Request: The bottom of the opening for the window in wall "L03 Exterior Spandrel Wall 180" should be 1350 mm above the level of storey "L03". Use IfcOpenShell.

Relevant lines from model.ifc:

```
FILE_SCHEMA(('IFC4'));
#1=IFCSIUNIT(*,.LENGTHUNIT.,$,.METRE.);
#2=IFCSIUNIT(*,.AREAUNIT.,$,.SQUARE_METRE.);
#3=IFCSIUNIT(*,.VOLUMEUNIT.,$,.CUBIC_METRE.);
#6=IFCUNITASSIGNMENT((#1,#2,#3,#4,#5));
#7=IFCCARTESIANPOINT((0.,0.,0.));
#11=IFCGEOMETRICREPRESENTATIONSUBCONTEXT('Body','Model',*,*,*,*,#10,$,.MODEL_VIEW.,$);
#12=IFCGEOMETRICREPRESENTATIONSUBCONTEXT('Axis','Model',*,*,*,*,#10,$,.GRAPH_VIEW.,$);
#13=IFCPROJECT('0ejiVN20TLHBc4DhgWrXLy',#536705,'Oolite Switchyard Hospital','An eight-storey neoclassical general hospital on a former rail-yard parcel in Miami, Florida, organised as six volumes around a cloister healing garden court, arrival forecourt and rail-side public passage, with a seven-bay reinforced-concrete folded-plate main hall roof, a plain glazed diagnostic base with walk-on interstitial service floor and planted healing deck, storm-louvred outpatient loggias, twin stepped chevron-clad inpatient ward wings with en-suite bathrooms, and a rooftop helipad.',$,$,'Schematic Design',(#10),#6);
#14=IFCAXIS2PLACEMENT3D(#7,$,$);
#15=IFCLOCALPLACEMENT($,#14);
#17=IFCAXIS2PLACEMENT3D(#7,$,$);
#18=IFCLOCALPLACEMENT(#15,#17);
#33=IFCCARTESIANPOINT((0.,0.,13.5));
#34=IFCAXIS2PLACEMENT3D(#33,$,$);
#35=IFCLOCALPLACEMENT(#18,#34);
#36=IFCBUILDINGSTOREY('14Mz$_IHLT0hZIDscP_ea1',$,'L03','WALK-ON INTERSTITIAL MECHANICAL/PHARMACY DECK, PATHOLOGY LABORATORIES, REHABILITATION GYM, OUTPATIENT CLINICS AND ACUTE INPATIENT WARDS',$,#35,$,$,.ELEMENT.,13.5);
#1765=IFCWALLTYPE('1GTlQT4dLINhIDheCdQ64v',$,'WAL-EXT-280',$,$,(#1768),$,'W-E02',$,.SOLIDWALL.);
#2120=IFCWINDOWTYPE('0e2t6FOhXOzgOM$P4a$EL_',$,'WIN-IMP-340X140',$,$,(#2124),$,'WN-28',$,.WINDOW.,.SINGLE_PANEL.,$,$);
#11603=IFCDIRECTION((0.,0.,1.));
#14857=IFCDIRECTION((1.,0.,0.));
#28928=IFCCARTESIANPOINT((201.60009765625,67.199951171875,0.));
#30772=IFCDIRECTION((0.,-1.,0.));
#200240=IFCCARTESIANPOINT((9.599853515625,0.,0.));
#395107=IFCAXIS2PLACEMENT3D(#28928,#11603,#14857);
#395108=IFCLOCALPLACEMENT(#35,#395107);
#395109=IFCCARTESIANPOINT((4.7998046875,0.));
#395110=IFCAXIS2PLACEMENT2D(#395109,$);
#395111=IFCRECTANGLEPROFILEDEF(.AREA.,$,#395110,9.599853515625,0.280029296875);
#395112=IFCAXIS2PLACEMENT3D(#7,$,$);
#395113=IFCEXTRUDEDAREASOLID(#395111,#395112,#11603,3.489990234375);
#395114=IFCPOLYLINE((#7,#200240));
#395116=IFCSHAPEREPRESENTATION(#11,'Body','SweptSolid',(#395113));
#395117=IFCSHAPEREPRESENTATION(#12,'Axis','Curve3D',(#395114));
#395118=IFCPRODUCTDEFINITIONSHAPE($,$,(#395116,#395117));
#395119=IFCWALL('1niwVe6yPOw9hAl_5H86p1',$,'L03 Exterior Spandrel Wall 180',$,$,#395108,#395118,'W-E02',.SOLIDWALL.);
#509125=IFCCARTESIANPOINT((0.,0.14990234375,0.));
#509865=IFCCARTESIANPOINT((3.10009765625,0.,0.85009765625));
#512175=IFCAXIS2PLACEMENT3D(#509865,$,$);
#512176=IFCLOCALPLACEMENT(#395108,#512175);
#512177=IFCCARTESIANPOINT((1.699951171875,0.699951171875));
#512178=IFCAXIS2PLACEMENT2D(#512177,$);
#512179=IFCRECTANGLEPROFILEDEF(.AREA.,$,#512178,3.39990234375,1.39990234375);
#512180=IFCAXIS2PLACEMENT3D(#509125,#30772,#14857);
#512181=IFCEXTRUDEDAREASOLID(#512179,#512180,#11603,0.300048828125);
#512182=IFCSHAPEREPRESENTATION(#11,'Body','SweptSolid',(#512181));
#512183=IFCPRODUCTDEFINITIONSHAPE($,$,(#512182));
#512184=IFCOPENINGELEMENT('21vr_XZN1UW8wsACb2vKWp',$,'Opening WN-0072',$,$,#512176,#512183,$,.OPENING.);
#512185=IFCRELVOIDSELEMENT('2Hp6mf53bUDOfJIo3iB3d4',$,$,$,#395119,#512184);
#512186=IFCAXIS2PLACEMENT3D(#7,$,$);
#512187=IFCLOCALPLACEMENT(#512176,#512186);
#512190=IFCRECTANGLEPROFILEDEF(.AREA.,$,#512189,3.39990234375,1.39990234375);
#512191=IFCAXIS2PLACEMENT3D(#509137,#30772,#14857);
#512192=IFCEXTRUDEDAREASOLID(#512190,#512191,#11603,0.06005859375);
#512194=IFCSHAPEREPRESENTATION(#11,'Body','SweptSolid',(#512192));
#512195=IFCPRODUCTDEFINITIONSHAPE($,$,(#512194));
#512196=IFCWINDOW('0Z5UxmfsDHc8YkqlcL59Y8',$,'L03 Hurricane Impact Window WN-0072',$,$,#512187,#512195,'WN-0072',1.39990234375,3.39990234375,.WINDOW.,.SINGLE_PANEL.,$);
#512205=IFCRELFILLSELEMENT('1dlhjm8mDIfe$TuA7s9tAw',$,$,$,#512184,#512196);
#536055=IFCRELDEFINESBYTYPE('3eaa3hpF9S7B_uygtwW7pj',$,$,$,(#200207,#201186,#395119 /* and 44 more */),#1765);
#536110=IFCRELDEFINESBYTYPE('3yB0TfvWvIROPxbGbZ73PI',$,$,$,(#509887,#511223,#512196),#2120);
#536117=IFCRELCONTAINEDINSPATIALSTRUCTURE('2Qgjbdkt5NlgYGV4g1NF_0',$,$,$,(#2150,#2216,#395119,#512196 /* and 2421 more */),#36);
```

```python
import numpy as np
import ifcopenshell
import ifcopenshell.api.geometry
import ifcopenshell.geom
import ifcopenshell.util.element
import ifcopenshell.util.placement
import ifcopenshell.util.shape
import ifcopenshell.util.unit

model = ifcopenshell.open("model.ifc")
unit_scale = ifcopenshell.util.unit.calculate_unit_scale(model)

window = model.by_id(512196)
opening = window.FillsVoids[0].RelatingOpeningElement
storey = ifcopenshell.util.element.get_container(window, ifc_class="IfcBuildingStorey")
level = ifcopenshell.util.placement.get_local_placement(storey.ObjectPlacement)[2, 3]

# The opening's origin need not be at the sill, so measure its lowest point.
shape = ifcopenshell.geom.create_shape(ifcopenshell.geom.settings(), opening)
bottom = ifcopenshell.util.shape.get_shape_bottom_elevation(shape, shape.geometry) / unit_scale
dz = level + 1.35 / unit_scale - bottom

shift = np.array([0.0, 0.0, dz])
# The window is placed relative to its opening, so it follows when the opening moves.
matrix = ifcopenshell.util.placement.get_local_placement(opening.ObjectPlacement)
matrix[:3, 3] += shift
ifcopenshell.api.geometry.edit_object_placement(
    model, product=opening, matrix=matrix, is_si=False, should_transform_children=True
)

print(f"moved by {dz * unit_scale:+.3f} m")

model.write("model_updated.ifc")
```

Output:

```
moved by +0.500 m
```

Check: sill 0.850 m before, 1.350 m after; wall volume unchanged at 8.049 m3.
